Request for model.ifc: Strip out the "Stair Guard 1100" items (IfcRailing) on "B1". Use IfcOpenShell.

First a look at what the model holds.

```python
import ifcopenshell
import ifcopenshell.util.element

model = ifcopenshell.open("model.ifc")
print(model.schema)
storey = next(s for s in model.by_type("IfcBuildingStorey") if s.Name == "B1")
railings = [e for e in ifcopenshell.util.element.get_decomposition(storey) if e.is_a("IfcRailing")]
seen = {}
for e in railings:
    element_type = ifcopenshell.util.element.get_type(e)
    name = element_type.Name if element_type not in (None, e) else None
    seen[name] = seen.get(name, 0) + 1
for name, count in sorted(seen.items(), key=str):
    print(count, "x", name)
```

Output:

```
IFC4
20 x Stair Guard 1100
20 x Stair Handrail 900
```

```python
import ifcopenshell
import ifcopenshell.api.root
import ifcopenshell.util.element

model = ifcopenshell.open("model.ifc")

storey = next(s for s in model.by_type("IfcBuildingStorey") if s.Name == "B1")
railings = [e for e in ifcopenshell.util.element.get_decomposition(storey) if e.is_a("IfcRailing")]
targets = [e for e in railings if (t := ifcopenshell.util.element.get_type(e)) not in (None, e) and t.Name == "Stair Guard 1100"]

for e in targets:
    ifcopenshell.api.root.remove_product(model, product=e)
print(len(targets), "removed")

model.write("model-out.ifc")
```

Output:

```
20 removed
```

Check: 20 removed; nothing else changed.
